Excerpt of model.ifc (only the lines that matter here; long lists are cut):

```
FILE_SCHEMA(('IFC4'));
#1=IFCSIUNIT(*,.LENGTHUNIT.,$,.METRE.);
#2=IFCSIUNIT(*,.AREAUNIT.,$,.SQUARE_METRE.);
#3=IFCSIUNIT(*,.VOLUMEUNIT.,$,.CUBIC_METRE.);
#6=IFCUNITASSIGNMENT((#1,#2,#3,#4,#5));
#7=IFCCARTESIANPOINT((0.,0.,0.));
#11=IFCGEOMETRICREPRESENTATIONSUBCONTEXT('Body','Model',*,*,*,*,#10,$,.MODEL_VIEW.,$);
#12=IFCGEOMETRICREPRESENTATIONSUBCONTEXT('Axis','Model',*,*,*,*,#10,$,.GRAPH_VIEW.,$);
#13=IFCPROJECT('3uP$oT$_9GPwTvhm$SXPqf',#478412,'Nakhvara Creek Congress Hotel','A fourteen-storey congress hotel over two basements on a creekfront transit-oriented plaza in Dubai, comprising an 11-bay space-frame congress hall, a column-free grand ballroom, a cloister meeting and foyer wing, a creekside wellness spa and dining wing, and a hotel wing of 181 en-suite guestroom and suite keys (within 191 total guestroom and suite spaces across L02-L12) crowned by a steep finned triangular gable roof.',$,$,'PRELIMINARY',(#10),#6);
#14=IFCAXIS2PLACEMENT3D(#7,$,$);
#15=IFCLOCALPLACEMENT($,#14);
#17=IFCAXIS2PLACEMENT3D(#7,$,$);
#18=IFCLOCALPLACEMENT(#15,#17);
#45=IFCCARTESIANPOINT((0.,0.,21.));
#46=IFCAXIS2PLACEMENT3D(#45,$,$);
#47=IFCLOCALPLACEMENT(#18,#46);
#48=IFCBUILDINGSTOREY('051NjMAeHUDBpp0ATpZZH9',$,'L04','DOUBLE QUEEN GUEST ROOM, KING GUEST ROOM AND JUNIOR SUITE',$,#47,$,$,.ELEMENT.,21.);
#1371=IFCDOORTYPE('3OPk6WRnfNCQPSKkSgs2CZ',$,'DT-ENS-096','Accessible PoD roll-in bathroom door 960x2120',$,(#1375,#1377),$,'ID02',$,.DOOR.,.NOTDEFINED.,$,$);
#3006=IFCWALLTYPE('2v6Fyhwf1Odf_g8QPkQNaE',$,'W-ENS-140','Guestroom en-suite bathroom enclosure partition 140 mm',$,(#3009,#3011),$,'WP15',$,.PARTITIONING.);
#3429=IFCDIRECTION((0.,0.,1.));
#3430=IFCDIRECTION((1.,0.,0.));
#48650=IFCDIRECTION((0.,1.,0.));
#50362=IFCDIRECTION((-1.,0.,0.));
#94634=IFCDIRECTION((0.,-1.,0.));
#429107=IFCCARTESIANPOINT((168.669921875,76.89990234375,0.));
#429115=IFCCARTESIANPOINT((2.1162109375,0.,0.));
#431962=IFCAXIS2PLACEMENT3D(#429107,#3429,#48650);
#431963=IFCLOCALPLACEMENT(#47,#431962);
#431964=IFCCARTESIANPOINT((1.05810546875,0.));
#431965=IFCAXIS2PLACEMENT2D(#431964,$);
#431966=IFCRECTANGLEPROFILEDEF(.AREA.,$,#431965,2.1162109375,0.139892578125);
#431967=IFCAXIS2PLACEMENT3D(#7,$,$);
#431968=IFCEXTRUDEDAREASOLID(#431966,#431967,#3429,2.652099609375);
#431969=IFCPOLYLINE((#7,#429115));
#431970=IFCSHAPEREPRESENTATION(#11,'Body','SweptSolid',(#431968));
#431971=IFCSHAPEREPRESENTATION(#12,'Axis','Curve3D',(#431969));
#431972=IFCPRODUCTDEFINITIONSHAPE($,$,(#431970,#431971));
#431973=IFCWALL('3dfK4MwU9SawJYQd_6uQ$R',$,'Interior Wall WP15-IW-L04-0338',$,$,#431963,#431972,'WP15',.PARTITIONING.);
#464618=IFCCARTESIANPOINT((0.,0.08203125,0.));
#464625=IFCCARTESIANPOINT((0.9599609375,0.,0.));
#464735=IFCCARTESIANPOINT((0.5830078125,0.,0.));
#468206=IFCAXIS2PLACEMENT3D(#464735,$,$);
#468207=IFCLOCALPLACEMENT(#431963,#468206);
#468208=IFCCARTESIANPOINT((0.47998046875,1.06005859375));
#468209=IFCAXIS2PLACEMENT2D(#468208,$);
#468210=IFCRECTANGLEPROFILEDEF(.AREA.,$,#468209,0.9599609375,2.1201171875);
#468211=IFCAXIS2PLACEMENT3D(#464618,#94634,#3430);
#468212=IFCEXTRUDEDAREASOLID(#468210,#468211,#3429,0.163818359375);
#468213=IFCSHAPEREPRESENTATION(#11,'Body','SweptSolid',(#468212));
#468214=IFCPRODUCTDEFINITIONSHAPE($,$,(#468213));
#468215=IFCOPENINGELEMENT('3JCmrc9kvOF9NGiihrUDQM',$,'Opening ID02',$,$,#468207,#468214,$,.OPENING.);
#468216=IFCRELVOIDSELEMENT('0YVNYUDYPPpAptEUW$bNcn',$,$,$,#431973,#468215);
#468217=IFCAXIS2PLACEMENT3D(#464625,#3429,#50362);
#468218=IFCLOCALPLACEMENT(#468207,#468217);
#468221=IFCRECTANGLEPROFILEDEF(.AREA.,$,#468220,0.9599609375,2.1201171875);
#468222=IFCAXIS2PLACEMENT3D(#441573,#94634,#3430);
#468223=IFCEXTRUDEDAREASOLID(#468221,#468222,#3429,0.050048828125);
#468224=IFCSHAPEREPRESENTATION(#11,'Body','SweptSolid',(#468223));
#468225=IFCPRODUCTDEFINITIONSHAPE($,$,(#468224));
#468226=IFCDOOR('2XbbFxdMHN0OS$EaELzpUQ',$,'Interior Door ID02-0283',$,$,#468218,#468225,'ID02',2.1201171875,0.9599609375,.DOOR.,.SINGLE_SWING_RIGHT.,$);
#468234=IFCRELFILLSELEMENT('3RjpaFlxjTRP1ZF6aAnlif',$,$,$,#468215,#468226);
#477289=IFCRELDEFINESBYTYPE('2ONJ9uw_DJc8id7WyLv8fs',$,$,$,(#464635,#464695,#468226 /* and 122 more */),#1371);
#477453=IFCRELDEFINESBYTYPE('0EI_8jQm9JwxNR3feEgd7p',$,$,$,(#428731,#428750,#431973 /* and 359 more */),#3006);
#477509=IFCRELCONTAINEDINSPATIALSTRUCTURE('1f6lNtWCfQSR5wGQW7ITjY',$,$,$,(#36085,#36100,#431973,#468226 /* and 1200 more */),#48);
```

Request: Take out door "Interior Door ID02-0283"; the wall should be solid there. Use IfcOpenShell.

```python
import ifcopenshell
import ifcopenshell.api.feature
import ifcopenshell.api.root
import ifcopenshell.geom
import ifcopenshell.util.shape

model = ifcopenshell.open("model.ifc")
settings = ifcopenshell.geom.settings()


def volume(element):
    """Net volume in cubic metres, openings subtracted."""
    shape = ifcopenshell.geom.create_shape(settings, element)
    return ifcopenshell.util.shape.get_volume(shape.geometry)


door = model.by_guid("2XbbFxdMHN0OS$EaELzpUQ")
opening = door.FillsVoids[0].RelatingOpeningElement
wall = opening.VoidsElements[0].RelatingBuildingElement
before = volume(wall)

ifcopenshell.api.root.remove_product(model, product=door)
ifcopenshell.api.feature.remove_feature(model, feature=opening)

after = volume(wall)

print(f"wall volume {before:.3f} -> {after:.3f} m3")

model.write("model_rev.ifc")
```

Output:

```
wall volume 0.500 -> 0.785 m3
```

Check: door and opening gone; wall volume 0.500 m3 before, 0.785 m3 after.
